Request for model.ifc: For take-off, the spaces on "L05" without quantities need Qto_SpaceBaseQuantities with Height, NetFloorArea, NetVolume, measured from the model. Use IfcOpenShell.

First a look at what the model holds.

```python
import ifcopenshell
import ifcopenshell.util.element
import ifcopenshell.util.unit

model = ifcopenshell.open("model.ifc")
print(model.schema)
for unit_type in ("LENGTHUNIT", "AREAUNIT", "VOLUMEUNIT"):
    print(unit_type, ifcopenshell.util.unit.calculate_unit_scale(model, unit_type))
storey = next(s for s in model.by_type("IfcBuildingStorey") if s.Name == "L05")
spaces = [e for e in ifcopenshell.util.element.get_decomposition(storey) if e.is_a("IfcSpace")]
for e in sorted(spaces, key=lambda e: e.id()):
    print(e.id(), e.is_a(), e.Name, list(ifcopenshell.util.element.get_psets(e, qtos_only=True)), sep=" | ")
```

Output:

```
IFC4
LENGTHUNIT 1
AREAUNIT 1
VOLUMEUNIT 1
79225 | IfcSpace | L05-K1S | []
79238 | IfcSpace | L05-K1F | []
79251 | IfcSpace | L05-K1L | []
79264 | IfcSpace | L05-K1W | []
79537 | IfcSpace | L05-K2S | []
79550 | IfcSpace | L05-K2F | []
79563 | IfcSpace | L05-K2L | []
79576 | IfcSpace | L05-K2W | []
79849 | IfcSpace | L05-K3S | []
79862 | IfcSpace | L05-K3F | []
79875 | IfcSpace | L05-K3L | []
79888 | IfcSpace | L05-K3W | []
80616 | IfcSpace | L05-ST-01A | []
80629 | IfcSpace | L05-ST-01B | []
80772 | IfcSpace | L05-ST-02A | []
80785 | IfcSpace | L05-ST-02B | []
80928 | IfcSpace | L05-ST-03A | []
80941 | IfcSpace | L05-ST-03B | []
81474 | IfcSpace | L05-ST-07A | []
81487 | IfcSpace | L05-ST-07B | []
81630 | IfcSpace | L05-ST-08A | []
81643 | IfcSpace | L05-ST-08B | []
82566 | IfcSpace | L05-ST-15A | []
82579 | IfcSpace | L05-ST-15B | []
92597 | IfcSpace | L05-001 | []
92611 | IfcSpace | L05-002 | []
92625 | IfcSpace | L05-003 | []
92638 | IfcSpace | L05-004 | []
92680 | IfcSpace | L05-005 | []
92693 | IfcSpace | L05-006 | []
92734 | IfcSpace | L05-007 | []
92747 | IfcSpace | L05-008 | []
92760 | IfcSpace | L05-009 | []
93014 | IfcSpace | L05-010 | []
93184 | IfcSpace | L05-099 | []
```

```python
import ifcopenshell
import ifcopenshell.api.pset
import ifcopenshell.geom
import ifcopenshell.util.element
import ifcopenshell.util.shape
import ifcopenshell.util.unit

model = ifcopenshell.open("model.ifc")
unit_scale = ifcopenshell.util.unit.calculate_unit_scale(model)
area_scale = ifcopenshell.util.unit.calculate_unit_scale(model, "AREAUNIT")
volume_scale = ifcopenshell.util.unit.calculate_unit_scale(model, "VOLUMEUNIT")
settings = ifcopenshell.geom.settings()

storey = next(s for s in model.by_type("IfcBuildingStorey") if s.Name == "L05")
spaces = [e for e in ifcopenshell.util.element.get_decomposition(storey) if e.is_a("IfcSpace")]

for e in sorted(spaces, key=lambda e: e.id()):
    if ifcopenshell.util.element.get_psets(e, qtos_only=True, should_inherit=False):
        continue
    # Geometry comes back in metres, in the element's own axes.
    shape = ifcopenshell.geom.create_shape(settings, e)
    values = {
        "Height": ifcopenshell.util.shape.get_z(shape.geometry) / unit_scale,
        "NetFloorArea": ifcopenshell.util.shape.get_footprint_area(shape.geometry) / area_scale,
        "NetVolume": ifcopenshell.util.shape.get_volume(shape.geometry) / volume_scale,
    }
    qto = ifcopenshell.api.pset.add_qto(model, product=e, name="Qto_SpaceBaseQuantities")
    ifcopenshell.api.pset.edit_qto(model, qto=qto, properties=values)
    print(e.id(), {k: round(v, 3) for k, v in values.items()})

model.write("model_rev.ifc")
```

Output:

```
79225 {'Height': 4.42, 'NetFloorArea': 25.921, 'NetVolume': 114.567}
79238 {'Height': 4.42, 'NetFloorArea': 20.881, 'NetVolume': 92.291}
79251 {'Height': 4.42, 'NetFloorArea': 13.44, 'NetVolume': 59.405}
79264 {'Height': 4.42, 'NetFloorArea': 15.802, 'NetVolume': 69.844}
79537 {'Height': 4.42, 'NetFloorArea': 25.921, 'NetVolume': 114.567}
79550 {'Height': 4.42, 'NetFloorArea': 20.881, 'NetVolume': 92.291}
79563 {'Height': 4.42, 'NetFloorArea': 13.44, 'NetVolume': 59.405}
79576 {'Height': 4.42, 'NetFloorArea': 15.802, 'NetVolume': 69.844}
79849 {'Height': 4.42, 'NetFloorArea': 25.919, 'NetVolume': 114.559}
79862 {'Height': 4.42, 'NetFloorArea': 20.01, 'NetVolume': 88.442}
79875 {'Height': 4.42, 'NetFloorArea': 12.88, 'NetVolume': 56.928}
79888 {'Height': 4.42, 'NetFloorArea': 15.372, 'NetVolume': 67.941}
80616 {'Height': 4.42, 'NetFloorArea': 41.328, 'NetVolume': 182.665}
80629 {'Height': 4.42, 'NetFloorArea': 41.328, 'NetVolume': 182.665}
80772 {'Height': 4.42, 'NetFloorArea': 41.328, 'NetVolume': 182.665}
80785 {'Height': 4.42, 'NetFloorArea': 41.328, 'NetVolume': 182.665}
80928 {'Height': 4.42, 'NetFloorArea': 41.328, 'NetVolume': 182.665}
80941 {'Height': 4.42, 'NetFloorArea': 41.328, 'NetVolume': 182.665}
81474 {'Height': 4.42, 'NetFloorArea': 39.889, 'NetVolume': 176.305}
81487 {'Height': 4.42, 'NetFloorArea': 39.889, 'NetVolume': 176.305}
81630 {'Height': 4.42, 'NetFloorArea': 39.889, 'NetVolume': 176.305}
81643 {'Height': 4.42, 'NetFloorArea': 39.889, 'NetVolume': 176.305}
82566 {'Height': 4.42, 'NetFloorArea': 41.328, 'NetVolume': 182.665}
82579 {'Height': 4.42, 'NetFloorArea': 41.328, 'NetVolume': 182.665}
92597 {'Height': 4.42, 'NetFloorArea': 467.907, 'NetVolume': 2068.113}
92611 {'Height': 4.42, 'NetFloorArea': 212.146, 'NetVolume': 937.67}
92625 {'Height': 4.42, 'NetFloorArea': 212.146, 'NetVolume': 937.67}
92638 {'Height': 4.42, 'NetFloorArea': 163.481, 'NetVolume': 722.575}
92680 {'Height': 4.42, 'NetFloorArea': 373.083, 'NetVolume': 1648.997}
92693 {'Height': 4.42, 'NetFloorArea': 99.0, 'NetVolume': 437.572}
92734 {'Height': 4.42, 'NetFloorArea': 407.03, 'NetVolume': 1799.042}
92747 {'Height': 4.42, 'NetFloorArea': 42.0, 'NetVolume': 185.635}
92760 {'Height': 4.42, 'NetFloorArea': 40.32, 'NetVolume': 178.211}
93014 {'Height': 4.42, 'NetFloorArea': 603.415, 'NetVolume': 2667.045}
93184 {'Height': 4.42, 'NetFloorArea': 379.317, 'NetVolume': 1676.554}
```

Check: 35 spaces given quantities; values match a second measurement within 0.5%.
